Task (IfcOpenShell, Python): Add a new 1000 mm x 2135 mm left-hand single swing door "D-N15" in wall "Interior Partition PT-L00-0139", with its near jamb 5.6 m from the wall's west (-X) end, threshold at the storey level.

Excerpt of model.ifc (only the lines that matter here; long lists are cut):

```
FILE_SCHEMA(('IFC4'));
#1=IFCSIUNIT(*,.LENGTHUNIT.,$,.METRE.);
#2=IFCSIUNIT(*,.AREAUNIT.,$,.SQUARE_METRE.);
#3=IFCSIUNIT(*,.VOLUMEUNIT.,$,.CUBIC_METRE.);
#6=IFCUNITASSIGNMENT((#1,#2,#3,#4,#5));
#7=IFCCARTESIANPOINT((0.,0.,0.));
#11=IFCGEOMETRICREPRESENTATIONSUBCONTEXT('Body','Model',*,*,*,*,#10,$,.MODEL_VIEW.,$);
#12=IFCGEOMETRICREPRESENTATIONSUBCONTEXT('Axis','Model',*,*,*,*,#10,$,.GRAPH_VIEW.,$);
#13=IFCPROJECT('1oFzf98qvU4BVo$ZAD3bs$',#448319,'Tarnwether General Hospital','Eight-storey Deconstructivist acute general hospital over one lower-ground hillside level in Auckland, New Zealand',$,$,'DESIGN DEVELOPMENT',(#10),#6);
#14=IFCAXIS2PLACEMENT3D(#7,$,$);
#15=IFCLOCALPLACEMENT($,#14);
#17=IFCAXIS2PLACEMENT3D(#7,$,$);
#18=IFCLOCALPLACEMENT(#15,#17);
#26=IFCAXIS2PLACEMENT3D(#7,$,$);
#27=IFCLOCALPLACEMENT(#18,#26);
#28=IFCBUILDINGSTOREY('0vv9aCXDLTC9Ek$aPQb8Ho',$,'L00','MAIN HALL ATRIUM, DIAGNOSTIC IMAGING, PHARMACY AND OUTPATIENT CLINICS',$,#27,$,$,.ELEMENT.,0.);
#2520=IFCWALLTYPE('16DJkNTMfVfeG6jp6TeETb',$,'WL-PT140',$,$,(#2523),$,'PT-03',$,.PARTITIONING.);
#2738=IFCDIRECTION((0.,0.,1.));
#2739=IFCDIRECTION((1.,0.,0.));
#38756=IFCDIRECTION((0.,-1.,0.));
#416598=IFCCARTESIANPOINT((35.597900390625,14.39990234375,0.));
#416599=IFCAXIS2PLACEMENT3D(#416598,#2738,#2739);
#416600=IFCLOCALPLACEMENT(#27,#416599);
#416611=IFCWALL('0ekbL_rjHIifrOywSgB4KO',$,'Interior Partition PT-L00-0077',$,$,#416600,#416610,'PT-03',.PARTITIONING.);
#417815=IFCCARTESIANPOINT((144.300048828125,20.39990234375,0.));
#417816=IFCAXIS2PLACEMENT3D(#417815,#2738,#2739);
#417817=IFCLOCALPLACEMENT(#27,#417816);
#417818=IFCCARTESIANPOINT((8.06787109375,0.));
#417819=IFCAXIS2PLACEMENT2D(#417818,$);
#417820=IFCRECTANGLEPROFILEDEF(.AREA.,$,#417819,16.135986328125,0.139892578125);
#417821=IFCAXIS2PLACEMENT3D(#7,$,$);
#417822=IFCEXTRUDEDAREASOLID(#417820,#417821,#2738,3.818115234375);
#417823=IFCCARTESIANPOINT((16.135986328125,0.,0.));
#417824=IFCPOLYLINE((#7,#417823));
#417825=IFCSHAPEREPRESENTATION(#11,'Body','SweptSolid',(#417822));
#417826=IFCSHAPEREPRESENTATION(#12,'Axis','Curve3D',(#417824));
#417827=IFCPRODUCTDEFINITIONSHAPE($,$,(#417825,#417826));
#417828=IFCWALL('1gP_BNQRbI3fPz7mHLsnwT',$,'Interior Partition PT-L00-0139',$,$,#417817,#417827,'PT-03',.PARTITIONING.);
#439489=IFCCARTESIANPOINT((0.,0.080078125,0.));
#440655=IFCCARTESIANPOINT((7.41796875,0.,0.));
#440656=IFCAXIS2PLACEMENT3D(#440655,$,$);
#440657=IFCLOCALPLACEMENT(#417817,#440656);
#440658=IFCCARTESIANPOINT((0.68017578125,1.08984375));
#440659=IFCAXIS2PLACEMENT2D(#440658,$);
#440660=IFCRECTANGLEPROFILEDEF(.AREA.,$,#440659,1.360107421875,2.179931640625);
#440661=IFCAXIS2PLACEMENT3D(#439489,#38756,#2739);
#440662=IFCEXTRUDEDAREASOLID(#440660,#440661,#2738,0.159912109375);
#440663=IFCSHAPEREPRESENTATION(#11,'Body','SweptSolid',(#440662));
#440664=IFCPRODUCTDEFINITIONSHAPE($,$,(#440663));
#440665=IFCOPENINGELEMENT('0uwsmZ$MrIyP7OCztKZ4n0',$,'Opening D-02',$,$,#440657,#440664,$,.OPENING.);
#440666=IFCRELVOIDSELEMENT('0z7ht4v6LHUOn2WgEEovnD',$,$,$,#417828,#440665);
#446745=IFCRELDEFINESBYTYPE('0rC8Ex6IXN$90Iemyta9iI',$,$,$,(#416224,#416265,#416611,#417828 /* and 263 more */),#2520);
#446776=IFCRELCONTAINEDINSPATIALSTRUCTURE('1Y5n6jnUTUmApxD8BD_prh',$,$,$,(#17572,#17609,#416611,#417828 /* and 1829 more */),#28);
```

```python
import numpy as np
import ifcopenshell
import ifcopenshell.api.feature
import ifcopenshell.api.geometry
import ifcopenshell.api.root
import ifcopenshell.api.spatial
import ifcopenshell.geom
import ifcopenshell.util.element
import ifcopenshell.util.placement
import ifcopenshell.util.representation
import ifcopenshell.util.shape
import ifcopenshell.util.unit

model = ifcopenshell.open("model.ifc")
unit_scale = ifcopenshell.util.unit.calculate_unit_scale(model)
settings = ifcopenshell.geom.settings()


def volume(element):
    """Net volume in cubic metres, openings subtracted."""
    shape = ifcopenshell.geom.create_shape(settings, element)
    return ifcopenshell.util.shape.get_volume(shape.geometry)


wall = model.by_guid("1gP_BNQRbI3fPz7mHLsnwT")
storey = ifcopenshell.util.element.get_container(wall, ifc_class="IfcBuildingStorey")
context = ifcopenshell.util.representation.get_context(model, "Model", "Body", "MODEL_VIEW")
before = volume(wall)

width, height, from_end, sill = 1, 2.135, 5.6, 0.0  # metres

# The wall runs along its own X axis, and the end named is its -X end.
wall_shape = ifcopenshell.geom.create_shape(settings, wall)
x, y, z = ifcopenshell.util.shape.get_vertices(wall_shape.geometry).T
start = x.min() + from_end
face, thickness = float(y.min()), float(y.max() - y.min())
wall_matrix = ifcopenshell.util.placement.get_local_placement(wall.ObjectPlacement)
level = ifcopenshell.util.placement.get_local_placement(storey.ObjectPlacement)[2, 3]


def in_wall(x, y):
    """Placement at x, y metres in the wall's axes, at sill height."""
    matrix = wall_matrix.copy()
    matrix[:, 3] = wall_matrix @ np.array([x / unit_scale, y / unit_scale, 0.0, 1.0])
    matrix[2, 3] = level + sill / unit_scale
    return matrix


# Opening: a box that overshoots both wall faces by 50 mm.
opening = ifcopenshell.api.root.create_entity(model, ifc_class="IfcOpeningElement", predefined_type="OPENING")
box = ifcopenshell.api.geometry.add_wall_representation(
    model, context=context, length=width, height=height, thickness=thickness + 0.1
)
ifcopenshell.api.geometry.assign_representation(model, product=opening, representation=box)
ifcopenshell.api.geometry.edit_object_placement(model, product=opening, matrix=in_wall(start, face - 0.05), is_si=False)
ifcopenshell.api.feature.add_feature(model, feature=opening, element=wall)

door = ifcopenshell.api.root.create_entity(model, ifc_class="IfcDoor", name="D-N15", predefined_type="DOOR")
door.OverallWidth, door.OverallHeight = width / unit_scale, height / unit_scale
door.OperationType = "SINGLE_SWING_LEFT"
body = ifcopenshell.api.geometry.add_door_representation(
    model,
    context=context,
    overall_width=door.OverallWidth,
    overall_height=door.OverallHeight,
    operation_type="SINGLE_SWING_LEFT",
    lining_properties={"LiningDepth": thickness / unit_scale, "ThresholdDepth": thickness / unit_scale},
)
ifcopenshell.api.geometry.assign_representation(model, product=door, representation=body)
ifcopenshell.api.spatial.assign_container(model, products=[door], relating_structure=storey)
ifcopenshell.api.feature.add_filling(model, opening=opening, element=door)

# The lining spans the wall, so the door starts at the wall face.
ifcopenshell.api.geometry.edit_object_placement(model, product=door, matrix=in_wall(start, face), is_si=False)

after = volume(wall)

print(f"wall volume {before:.3f} -> {after:.3f} m3")

model.write("model_rev.ifc")
```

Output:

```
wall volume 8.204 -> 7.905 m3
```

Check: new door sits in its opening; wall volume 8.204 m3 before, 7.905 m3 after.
